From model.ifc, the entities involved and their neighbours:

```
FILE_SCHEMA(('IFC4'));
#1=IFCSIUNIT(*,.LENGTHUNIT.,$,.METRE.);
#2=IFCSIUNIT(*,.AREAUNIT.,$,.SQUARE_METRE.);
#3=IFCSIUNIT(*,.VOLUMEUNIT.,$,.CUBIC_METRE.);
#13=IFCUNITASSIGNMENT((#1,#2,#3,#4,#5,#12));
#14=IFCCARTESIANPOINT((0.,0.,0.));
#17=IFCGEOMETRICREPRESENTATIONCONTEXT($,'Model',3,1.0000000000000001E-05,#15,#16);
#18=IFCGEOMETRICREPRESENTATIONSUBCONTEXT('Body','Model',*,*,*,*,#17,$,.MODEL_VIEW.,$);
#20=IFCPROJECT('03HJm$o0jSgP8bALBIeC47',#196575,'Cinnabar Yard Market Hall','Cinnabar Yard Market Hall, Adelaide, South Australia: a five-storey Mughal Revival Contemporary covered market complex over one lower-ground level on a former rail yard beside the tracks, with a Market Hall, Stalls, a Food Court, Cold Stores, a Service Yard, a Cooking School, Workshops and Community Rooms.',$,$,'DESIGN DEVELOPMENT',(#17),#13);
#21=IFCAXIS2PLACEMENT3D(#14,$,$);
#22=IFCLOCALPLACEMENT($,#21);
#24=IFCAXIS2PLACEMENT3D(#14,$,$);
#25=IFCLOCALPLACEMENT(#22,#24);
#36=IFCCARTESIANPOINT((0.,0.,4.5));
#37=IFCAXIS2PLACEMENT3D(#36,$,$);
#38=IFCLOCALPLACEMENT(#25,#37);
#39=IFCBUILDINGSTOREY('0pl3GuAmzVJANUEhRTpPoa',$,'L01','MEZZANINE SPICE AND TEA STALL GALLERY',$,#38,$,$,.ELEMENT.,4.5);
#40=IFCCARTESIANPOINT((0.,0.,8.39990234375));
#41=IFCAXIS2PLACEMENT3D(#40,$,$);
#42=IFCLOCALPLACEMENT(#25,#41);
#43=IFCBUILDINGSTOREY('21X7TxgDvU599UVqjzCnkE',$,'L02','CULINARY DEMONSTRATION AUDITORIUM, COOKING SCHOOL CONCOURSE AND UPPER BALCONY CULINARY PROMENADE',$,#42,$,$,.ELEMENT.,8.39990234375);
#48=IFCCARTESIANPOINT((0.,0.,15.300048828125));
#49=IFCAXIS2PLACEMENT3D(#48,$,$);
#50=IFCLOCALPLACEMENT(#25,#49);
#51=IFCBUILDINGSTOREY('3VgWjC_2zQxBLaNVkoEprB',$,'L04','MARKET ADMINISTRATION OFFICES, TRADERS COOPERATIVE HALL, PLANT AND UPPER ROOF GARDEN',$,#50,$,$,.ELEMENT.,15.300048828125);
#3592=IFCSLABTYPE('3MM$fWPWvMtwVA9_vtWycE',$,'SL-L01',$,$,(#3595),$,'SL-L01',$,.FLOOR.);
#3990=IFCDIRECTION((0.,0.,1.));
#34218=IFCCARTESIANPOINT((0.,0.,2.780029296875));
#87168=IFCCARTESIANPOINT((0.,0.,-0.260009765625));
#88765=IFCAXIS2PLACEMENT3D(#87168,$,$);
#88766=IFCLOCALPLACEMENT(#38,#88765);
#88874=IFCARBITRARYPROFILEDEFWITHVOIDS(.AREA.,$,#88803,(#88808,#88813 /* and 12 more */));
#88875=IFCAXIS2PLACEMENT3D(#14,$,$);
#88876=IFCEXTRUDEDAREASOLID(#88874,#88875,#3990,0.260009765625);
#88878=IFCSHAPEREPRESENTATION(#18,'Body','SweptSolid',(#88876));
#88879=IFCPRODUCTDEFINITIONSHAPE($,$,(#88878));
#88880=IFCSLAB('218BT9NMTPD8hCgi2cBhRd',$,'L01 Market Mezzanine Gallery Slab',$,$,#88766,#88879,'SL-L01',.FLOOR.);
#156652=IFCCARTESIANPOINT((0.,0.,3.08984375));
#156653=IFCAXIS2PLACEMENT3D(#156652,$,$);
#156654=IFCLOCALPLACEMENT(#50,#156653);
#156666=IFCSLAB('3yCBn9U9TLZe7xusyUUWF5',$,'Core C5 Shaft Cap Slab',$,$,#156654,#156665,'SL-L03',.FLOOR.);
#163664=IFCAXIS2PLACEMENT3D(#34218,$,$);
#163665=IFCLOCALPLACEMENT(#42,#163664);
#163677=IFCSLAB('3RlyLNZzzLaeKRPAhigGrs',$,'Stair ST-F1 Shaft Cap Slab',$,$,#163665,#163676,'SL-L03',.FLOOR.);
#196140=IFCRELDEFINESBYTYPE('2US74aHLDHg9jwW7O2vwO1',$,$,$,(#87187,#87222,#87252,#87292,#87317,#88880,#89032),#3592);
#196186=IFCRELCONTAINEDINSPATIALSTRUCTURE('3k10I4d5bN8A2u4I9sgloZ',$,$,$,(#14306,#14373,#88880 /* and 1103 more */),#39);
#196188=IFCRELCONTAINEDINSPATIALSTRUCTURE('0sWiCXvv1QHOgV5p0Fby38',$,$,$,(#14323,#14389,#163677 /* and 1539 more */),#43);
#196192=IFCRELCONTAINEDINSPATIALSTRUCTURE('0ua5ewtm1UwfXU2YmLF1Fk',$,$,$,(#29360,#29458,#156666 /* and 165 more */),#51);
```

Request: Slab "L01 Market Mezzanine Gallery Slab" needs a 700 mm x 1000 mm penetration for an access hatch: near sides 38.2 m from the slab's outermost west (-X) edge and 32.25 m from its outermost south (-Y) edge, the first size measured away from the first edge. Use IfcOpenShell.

```python
import numpy as np
import ifcopenshell
import ifcopenshell.api.feature
import ifcopenshell.api.geometry
import ifcopenshell.api.root
import ifcopenshell.geom
import ifcopenshell.util.placement
import ifcopenshell.util.representation
import ifcopenshell.util.shape
import ifcopenshell.util.unit

model = ifcopenshell.open("model.ifc")
unit_scale = ifcopenshell.util.unit.calculate_unit_scale(model)
settings = ifcopenshell.geom.settings()


def volume(element):
    """Net volume in cubic metres, openings subtracted."""
    shape = ifcopenshell.geom.create_shape(settings, element)
    return ifcopenshell.util.shape.get_volume(shape.geometry)


slab = model.by_guid("218BT9NMTPD8hCgi2cBhRd")
before = volume(slab)

# Extent in the slab's own axes, in metres. The edges named are its -X and -Y sides.
slab_shape = ifcopenshell.geom.create_shape(settings, slab)
vertices = ifcopenshell.util.shape.get_vertices(slab_shape.geometry)
x_min, y_min, bottom = vertices.min(axis=0)
top = vertices[:, 2].max()

opening = ifcopenshell.api.root.create_entity(model, ifc_class="IfcOpeningElement", name="Access hatch opening", predefined_type="OPENING")
context = ifcopenshell.util.representation.get_context(model, "Model", "Body", "MODEL_VIEW")
width, depth = 0.7, 1
outline = [(0.0, 0.0), (width, 0.0), (width, depth), (0.0, depth), (0.0, 0.0)]
# Overshoot both faces by 50 mm so the cut is clean.
shape = ifcopenshell.api.geometry.add_slab_representation(
    model, context=context, depth=top - bottom + 0.1, polyline=outline
)
ifcopenshell.api.geometry.assign_representation(model, product=opening, representation=shape)

matrix = ifcopenshell.util.placement.get_local_placement(slab.ObjectPlacement)
matrix[:, 3] = matrix @ np.append(np.array([x_min + 38.2, y_min + 32.25, bottom - 0.05]) / unit_scale, 1.0)
ifcopenshell.api.geometry.edit_object_placement(model, product=opening, matrix=matrix, is_si=False)
ifcopenshell.api.feature.add_feature(model, feature=opening, element=slab)

after = volume(slab)

print(f"slab volume {before:.3f} -> {after:.3f} m3")

model.write("model_edited.ifc")
```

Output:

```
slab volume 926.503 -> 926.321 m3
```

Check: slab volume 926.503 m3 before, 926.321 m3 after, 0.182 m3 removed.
